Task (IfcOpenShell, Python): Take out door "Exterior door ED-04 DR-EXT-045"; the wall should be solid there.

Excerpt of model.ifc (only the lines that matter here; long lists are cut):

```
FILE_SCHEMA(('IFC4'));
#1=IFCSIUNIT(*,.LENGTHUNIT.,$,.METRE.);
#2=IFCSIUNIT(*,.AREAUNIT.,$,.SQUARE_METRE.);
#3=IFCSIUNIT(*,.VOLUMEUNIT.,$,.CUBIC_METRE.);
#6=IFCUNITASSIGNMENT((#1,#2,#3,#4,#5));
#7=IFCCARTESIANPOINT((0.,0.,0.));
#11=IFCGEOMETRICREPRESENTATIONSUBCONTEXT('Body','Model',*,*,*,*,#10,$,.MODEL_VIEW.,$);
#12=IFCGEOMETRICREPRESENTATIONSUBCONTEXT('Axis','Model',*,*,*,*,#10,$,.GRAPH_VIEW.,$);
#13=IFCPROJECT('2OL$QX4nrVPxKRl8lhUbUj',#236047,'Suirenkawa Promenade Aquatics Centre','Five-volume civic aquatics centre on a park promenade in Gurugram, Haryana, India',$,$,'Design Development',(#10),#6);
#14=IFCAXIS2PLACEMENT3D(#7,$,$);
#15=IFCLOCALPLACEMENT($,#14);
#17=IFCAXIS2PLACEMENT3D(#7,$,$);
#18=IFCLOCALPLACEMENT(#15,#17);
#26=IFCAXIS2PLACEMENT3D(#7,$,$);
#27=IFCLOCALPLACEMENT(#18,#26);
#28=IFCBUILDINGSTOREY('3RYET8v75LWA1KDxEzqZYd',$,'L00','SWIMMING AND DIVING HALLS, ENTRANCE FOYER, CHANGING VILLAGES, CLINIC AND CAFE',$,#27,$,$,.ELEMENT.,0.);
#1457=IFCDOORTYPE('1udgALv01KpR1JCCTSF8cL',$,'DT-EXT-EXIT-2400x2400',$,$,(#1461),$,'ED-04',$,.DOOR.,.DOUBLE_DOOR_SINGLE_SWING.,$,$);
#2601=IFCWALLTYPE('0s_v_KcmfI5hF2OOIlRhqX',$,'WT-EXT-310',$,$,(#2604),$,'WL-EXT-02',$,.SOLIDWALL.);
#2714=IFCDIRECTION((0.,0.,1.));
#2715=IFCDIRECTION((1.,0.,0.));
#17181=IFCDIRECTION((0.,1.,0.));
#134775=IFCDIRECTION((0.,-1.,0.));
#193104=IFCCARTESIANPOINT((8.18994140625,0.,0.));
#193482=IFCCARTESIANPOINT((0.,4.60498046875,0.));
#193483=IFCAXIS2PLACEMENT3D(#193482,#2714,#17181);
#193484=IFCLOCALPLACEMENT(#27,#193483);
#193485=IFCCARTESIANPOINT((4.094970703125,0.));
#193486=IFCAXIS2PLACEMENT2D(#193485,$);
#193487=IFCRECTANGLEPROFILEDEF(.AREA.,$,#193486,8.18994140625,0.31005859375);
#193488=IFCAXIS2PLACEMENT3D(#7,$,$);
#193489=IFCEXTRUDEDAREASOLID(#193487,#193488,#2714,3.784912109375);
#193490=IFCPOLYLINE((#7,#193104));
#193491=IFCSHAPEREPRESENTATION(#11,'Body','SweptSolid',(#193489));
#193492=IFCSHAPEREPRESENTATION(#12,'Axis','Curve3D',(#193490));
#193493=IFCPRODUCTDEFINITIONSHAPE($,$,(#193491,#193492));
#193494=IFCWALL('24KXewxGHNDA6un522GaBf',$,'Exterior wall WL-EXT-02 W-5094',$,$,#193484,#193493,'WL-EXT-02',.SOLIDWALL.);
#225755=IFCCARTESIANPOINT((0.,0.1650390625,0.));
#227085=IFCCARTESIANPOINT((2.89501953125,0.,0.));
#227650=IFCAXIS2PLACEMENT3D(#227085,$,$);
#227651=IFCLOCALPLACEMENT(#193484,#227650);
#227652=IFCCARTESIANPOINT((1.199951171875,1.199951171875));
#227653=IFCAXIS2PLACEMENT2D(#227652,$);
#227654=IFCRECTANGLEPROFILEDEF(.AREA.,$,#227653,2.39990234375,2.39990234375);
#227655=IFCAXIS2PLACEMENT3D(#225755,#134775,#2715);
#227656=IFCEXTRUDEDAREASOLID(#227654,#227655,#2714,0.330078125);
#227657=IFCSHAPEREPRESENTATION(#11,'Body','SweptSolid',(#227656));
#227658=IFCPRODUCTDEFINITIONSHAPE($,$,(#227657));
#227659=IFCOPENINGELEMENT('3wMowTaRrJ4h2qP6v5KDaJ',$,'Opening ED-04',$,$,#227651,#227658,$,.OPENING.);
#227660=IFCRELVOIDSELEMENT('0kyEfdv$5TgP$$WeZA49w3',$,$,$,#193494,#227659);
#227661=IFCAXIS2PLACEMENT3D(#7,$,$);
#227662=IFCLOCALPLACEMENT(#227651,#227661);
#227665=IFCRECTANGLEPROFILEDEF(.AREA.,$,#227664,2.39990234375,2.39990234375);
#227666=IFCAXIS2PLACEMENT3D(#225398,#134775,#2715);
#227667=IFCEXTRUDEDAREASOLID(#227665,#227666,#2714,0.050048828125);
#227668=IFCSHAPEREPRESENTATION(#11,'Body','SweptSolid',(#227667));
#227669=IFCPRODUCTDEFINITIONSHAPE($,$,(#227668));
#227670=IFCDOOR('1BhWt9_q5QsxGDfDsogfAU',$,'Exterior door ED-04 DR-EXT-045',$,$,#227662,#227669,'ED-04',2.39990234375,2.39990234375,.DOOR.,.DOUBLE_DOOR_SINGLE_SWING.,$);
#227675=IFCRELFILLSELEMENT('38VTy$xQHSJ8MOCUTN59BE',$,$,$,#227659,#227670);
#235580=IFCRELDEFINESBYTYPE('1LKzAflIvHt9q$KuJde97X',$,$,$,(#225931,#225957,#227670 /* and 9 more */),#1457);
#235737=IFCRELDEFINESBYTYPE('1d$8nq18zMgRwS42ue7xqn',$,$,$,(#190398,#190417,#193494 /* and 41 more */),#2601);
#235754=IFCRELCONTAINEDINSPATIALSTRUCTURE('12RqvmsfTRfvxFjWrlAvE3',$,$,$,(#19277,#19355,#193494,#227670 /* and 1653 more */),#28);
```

```python
import ifcopenshell
import ifcopenshell.api.feature
import ifcopenshell.api.root
import ifcopenshell.geom
import ifcopenshell.util.shape

model = ifcopenshell.open("model.ifc")
settings = ifcopenshell.geom.settings()


def volume(element):
    """Net volume in cubic metres, openings subtracted."""
    shape = ifcopenshell.geom.create_shape(settings, element)
    return ifcopenshell.util.shape.get_volume(shape.geometry)


door = model.by_guid("1BhWt9_q5QsxGDfDsogfAU")
opening = door.FillsVoids[0].RelatingOpeningElement
wall = opening.VoidsElements[0].RelatingBuildingElement
before = volume(wall)

ifcopenshell.api.root.remove_product(model, product=door)
ifcopenshell.api.feature.remove_feature(model, feature=opening)

after = volume(wall)

print(f"wall volume {before:.3f} -> {after:.3f} m3")

model.write("model_updated.ifc")
```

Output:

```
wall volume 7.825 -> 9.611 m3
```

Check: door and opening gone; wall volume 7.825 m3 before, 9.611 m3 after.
